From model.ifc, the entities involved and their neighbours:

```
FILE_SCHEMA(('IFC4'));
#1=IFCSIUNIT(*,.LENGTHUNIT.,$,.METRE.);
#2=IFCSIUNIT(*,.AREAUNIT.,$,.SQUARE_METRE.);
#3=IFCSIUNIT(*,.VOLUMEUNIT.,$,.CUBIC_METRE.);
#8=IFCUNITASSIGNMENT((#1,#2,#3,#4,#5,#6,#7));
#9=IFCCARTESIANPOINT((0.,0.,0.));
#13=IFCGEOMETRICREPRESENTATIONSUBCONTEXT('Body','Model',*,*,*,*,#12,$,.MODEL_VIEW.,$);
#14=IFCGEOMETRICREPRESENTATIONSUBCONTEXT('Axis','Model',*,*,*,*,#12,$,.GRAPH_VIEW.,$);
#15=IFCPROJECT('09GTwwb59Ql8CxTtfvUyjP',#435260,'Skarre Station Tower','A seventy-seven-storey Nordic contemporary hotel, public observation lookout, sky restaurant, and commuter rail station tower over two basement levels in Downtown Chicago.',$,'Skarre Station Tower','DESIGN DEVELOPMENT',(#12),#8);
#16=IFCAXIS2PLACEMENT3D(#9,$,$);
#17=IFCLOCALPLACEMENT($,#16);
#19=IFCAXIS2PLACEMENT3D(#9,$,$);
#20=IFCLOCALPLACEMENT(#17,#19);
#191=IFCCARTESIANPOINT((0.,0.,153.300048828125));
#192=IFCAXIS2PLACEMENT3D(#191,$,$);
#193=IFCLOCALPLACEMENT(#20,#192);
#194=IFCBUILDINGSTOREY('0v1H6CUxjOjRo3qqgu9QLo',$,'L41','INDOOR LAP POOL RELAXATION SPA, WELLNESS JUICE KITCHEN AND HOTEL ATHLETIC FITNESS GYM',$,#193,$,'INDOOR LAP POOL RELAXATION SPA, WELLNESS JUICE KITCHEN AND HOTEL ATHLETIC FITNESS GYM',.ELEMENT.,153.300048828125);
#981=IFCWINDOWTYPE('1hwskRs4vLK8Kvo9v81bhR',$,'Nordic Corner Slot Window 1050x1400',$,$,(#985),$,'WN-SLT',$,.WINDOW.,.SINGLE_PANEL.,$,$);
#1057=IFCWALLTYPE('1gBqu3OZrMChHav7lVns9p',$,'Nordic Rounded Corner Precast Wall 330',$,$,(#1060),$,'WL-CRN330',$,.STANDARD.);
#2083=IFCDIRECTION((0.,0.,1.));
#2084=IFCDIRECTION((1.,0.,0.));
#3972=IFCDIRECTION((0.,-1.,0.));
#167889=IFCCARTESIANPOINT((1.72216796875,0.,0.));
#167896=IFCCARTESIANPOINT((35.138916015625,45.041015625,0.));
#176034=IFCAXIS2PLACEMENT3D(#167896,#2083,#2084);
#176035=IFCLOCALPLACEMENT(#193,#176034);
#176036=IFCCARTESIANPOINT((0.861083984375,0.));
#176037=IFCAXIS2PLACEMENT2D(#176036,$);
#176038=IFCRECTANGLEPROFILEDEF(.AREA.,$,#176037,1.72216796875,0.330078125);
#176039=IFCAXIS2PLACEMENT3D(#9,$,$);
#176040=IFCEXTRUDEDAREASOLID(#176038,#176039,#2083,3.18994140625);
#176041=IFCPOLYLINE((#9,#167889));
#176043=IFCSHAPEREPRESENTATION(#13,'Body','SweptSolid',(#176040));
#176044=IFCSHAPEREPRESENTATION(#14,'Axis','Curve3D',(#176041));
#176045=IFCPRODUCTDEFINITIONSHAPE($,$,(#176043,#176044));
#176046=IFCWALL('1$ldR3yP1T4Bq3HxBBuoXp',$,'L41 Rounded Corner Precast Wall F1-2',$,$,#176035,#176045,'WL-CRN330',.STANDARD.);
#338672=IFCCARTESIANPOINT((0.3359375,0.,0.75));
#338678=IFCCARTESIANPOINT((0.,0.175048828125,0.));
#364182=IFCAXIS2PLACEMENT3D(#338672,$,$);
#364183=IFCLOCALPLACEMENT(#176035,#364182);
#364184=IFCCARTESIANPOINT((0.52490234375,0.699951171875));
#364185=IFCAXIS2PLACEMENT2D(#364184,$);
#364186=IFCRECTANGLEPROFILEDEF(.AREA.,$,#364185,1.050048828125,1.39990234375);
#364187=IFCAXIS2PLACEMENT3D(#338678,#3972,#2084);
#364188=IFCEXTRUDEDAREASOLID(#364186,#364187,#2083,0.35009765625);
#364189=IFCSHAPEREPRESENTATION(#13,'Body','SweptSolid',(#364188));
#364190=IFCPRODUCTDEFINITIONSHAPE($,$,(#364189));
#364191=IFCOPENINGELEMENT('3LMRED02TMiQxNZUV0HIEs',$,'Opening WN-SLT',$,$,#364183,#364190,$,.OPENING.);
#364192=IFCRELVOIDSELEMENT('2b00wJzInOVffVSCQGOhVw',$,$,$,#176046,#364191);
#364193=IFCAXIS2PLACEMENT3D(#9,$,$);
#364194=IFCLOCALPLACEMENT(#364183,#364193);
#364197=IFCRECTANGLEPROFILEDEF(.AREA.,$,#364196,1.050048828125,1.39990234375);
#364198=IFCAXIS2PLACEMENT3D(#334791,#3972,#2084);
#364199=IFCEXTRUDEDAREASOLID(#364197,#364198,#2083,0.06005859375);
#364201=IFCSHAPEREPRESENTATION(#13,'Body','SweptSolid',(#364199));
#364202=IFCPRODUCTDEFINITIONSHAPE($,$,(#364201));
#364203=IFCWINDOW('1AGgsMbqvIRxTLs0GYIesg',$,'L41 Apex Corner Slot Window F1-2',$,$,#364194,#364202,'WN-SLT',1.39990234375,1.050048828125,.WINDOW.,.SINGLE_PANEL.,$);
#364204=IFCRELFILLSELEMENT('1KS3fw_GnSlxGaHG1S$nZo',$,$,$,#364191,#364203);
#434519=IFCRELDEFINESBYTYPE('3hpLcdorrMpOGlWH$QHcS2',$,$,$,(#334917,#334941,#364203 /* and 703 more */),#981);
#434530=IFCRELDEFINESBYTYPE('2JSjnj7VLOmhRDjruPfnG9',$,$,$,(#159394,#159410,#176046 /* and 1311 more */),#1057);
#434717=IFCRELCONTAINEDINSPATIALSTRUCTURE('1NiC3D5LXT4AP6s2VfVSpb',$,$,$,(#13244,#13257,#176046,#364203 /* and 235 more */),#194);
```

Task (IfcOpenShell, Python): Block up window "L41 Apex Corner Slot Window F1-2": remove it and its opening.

```python
import ifcopenshell
import ifcopenshell.api.feature
import ifcopenshell.api.root
import ifcopenshell.geom
import ifcopenshell.util.shape

model = ifcopenshell.open("model.ifc")
settings = ifcopenshell.geom.settings()


def volume(element):
    """Net volume in cubic metres, openings subtracted."""
    shape = ifcopenshell.geom.create_shape(settings, element)
    return ifcopenshell.util.shape.get_volume(shape.geometry)


window = model.by_guid("1AGgsMbqvIRxTLs0GYIesg")
opening = window.FillsVoids[0].RelatingOpeningElement
wall = opening.VoidsElements[0].RelatingBuildingElement
before = volume(wall)

ifcopenshell.api.root.remove_product(model, product=window)
ifcopenshell.api.feature.remove_feature(model, feature=opening)

after = volume(wall)

print(f"wall volume {before:.3f} -> {after:.3f} m3")

model.write("model_v2.ifc")
```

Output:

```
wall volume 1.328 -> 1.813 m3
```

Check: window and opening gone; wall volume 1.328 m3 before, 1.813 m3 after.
